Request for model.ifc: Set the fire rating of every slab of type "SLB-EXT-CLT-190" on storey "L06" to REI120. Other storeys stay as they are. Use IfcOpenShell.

First a look at what the model holds.

```python
import ifcopenshell
import ifcopenshell.util.element

model = ifcopenshell.open("model.ifc")
print(model.schema)
storey = next(s for s in model.by_type("IfcBuildingStorey") if s.Name == "L06")
slabs = [e for e in ifcopenshell.util.element.get_decomposition(storey) if e.is_a("IfcSlab")]
seen = {}
for e in slabs:
    element_type = ifcopenshell.util.element.get_type(e)
    key = (element_type.Name if element_type != e and element_type else None, ifcopenshell.util.element.get_pset(e, "Pset_SlabCommon", "FireRating"))
    seen[key] = seen.get(key, 0) + 1
for (name, value), count in sorted(seen.items(), key=str):
    print(count, "x", name, "|", value)
```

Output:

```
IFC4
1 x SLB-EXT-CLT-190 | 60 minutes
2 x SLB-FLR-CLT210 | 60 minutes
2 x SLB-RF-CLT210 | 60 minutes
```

```python
import ifcopenshell
import ifcopenshell.api.pset
import ifcopenshell.util.element

model = ifcopenshell.open("model.ifc")

storey = next(s for s in model.by_type("IfcBuildingStorey") if s.Name == "L06")
slabs = [e for e in ifcopenshell.util.element.get_decomposition(storey) if e.is_a("IfcSlab")]

count = 0
for e in slabs:
    element_type = ifcopenshell.util.element.get_type(e)
    if element_type in (None, e) or element_type.Name != "SLB-EXT-CLT-190":
        continue
    # add_pset returns the element's existing set when there is one.
    pset = ifcopenshell.api.pset.add_pset(model, product=e, name="Pset_SlabCommon")
    ifcopenshell.api.pset.edit_pset(model, pset=pset, properties={"FireRating": "REI120"})
    count += 1

print(count, "slabs updated")

model.write("model_updated.ifc")
```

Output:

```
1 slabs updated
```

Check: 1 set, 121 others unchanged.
